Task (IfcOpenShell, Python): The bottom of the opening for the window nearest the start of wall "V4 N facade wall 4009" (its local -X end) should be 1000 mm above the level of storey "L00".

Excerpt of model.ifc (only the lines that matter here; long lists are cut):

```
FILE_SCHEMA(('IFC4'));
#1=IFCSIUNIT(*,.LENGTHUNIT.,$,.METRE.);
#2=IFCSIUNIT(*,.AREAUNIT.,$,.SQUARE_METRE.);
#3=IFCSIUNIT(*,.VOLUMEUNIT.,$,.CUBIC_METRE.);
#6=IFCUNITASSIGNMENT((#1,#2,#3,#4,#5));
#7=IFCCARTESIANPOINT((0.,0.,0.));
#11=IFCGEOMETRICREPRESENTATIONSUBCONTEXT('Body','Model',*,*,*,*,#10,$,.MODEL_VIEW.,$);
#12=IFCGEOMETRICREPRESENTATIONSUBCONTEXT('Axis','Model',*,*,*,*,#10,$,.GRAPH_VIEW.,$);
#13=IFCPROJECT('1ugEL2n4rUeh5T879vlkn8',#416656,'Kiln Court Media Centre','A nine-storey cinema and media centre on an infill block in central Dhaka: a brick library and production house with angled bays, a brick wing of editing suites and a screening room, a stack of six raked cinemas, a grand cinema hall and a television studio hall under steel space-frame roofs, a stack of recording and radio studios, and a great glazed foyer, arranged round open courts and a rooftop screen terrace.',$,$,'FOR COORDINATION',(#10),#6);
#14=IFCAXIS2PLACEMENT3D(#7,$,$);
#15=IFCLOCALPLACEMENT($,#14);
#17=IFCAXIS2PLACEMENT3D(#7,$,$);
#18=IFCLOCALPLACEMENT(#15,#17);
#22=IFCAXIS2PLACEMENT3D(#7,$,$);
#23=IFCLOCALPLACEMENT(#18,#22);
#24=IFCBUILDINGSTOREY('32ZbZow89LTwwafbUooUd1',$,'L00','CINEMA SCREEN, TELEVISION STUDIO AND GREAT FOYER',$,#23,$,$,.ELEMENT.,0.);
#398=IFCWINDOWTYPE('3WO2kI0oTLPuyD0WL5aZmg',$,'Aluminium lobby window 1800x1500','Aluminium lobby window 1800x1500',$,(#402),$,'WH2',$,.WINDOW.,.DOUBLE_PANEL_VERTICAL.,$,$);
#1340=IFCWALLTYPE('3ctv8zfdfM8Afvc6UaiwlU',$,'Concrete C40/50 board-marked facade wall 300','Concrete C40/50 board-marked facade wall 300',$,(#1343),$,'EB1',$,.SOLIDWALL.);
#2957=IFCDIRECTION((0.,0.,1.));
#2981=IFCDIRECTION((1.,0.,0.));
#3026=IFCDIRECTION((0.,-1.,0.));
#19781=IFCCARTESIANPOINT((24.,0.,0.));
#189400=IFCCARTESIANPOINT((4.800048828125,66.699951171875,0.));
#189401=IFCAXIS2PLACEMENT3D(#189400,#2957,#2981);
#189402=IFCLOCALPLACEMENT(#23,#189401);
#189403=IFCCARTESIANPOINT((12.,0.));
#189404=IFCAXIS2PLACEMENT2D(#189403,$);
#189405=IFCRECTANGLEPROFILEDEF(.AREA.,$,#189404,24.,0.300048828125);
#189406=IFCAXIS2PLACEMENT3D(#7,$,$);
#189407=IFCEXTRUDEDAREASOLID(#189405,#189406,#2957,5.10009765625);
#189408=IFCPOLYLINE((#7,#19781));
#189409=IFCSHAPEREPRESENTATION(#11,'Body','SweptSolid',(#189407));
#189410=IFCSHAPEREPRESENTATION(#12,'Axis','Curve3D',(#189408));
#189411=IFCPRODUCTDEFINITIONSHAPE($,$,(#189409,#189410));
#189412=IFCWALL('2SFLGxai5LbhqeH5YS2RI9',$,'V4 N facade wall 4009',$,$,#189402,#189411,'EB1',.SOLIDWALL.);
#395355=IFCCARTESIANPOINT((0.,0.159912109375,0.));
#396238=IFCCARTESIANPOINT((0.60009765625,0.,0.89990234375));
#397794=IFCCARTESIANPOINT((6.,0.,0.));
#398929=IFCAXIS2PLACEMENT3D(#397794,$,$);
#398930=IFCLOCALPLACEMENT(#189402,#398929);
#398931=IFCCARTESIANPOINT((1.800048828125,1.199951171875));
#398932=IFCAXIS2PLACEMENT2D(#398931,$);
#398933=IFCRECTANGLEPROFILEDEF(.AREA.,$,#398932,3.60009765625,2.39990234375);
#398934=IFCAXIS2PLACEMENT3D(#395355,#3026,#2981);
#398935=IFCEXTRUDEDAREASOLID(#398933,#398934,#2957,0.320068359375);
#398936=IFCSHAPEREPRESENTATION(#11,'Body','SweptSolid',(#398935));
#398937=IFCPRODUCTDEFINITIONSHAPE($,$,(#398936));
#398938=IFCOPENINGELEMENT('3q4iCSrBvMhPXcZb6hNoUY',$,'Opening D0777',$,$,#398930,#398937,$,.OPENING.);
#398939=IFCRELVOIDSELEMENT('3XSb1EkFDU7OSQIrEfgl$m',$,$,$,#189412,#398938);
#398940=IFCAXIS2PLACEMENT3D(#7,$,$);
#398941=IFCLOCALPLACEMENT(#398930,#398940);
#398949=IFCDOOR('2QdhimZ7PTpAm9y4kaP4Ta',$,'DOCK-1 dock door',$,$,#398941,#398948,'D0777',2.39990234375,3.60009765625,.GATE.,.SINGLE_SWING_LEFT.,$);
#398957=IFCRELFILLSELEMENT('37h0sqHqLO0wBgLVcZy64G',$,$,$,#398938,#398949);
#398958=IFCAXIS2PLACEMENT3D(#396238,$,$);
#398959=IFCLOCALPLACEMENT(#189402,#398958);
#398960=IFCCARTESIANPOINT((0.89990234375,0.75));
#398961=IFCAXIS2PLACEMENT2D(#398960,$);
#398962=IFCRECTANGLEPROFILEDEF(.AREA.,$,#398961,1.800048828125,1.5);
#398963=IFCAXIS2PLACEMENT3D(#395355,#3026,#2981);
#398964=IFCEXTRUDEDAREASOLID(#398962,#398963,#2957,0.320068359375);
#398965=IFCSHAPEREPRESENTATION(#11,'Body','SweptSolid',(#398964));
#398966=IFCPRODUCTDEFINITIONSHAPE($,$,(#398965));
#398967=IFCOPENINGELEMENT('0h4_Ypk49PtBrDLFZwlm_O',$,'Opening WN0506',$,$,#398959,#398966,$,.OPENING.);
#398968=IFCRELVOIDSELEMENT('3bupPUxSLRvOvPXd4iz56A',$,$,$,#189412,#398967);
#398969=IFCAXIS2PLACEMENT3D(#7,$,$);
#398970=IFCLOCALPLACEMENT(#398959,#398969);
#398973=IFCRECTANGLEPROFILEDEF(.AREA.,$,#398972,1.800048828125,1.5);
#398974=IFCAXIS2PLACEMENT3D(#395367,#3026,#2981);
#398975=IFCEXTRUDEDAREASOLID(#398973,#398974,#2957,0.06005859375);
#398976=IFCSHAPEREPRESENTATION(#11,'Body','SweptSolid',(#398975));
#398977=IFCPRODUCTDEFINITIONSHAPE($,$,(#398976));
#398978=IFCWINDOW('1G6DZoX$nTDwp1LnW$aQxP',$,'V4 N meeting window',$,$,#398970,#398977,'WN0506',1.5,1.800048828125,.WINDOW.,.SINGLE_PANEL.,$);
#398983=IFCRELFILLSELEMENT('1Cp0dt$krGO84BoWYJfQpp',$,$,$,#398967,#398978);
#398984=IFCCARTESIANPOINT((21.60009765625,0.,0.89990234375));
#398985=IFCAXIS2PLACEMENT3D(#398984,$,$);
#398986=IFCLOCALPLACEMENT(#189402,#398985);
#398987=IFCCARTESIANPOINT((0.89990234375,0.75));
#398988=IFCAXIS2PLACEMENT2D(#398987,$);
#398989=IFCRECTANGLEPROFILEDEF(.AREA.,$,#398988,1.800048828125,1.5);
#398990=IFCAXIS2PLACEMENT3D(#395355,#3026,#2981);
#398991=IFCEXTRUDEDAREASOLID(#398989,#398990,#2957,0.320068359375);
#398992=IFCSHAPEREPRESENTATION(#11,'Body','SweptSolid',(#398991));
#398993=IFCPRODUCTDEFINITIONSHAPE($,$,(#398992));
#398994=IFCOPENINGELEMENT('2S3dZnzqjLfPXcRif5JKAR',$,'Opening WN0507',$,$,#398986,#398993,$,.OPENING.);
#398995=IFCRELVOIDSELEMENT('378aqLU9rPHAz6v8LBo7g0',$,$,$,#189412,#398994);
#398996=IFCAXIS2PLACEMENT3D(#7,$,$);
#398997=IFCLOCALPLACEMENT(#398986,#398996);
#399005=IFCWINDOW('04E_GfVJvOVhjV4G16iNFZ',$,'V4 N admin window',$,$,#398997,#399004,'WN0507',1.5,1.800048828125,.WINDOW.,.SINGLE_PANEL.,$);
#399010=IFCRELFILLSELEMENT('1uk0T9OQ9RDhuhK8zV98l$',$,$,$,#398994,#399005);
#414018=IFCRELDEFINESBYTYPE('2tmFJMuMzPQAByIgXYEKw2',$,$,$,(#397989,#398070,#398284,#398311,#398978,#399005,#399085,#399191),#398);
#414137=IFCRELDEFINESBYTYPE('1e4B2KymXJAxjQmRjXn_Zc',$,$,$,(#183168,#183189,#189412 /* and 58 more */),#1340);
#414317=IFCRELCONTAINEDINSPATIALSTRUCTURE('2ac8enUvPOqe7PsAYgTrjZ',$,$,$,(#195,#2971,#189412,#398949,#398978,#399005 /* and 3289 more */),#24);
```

```python
import numpy as np
import ifcopenshell
import ifcopenshell.api.geometry
import ifcopenshell.geom
import ifcopenshell.util.element
import ifcopenshell.util.placement
import ifcopenshell.util.shape
import ifcopenshell.util.unit

model = ifcopenshell.open("model.ifc")
unit_scale = ifcopenshell.util.unit.calculate_unit_scale(model)

window = model.by_guid("1G6DZoX$nTDwp1LnW$aQxP")
opening = window.FillsVoids[0].RelatingOpeningElement
storey = ifcopenshell.util.element.get_container(window, ifc_class="IfcBuildingStorey")
level = ifcopenshell.util.placement.get_local_placement(storey.ObjectPlacement)[2, 3]

# The opening's origin need not be at the sill, so measure its lowest point.
shape = ifcopenshell.geom.create_shape(ifcopenshell.geom.settings(), opening)
bottom = ifcopenshell.util.shape.get_shape_bottom_elevation(shape, shape.geometry) / unit_scale
dz = level + 1 / unit_scale - bottom

shift = np.array([0.0, 0.0, dz])
# The window is placed relative to its opening, so it follows when the opening moves.
matrix = ifcopenshell.util.placement.get_local_placement(opening.ObjectPlacement)
matrix[:3, 3] += shift
ifcopenshell.api.geometry.edit_object_placement(
    model, product=opening, matrix=matrix, is_si=False, should_transform_children=True
)

print(f"moved by {dz * unit_scale:+.3f} m")

model.write("model_rev.ifc")
```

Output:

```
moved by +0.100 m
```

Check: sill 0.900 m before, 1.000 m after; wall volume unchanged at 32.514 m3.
